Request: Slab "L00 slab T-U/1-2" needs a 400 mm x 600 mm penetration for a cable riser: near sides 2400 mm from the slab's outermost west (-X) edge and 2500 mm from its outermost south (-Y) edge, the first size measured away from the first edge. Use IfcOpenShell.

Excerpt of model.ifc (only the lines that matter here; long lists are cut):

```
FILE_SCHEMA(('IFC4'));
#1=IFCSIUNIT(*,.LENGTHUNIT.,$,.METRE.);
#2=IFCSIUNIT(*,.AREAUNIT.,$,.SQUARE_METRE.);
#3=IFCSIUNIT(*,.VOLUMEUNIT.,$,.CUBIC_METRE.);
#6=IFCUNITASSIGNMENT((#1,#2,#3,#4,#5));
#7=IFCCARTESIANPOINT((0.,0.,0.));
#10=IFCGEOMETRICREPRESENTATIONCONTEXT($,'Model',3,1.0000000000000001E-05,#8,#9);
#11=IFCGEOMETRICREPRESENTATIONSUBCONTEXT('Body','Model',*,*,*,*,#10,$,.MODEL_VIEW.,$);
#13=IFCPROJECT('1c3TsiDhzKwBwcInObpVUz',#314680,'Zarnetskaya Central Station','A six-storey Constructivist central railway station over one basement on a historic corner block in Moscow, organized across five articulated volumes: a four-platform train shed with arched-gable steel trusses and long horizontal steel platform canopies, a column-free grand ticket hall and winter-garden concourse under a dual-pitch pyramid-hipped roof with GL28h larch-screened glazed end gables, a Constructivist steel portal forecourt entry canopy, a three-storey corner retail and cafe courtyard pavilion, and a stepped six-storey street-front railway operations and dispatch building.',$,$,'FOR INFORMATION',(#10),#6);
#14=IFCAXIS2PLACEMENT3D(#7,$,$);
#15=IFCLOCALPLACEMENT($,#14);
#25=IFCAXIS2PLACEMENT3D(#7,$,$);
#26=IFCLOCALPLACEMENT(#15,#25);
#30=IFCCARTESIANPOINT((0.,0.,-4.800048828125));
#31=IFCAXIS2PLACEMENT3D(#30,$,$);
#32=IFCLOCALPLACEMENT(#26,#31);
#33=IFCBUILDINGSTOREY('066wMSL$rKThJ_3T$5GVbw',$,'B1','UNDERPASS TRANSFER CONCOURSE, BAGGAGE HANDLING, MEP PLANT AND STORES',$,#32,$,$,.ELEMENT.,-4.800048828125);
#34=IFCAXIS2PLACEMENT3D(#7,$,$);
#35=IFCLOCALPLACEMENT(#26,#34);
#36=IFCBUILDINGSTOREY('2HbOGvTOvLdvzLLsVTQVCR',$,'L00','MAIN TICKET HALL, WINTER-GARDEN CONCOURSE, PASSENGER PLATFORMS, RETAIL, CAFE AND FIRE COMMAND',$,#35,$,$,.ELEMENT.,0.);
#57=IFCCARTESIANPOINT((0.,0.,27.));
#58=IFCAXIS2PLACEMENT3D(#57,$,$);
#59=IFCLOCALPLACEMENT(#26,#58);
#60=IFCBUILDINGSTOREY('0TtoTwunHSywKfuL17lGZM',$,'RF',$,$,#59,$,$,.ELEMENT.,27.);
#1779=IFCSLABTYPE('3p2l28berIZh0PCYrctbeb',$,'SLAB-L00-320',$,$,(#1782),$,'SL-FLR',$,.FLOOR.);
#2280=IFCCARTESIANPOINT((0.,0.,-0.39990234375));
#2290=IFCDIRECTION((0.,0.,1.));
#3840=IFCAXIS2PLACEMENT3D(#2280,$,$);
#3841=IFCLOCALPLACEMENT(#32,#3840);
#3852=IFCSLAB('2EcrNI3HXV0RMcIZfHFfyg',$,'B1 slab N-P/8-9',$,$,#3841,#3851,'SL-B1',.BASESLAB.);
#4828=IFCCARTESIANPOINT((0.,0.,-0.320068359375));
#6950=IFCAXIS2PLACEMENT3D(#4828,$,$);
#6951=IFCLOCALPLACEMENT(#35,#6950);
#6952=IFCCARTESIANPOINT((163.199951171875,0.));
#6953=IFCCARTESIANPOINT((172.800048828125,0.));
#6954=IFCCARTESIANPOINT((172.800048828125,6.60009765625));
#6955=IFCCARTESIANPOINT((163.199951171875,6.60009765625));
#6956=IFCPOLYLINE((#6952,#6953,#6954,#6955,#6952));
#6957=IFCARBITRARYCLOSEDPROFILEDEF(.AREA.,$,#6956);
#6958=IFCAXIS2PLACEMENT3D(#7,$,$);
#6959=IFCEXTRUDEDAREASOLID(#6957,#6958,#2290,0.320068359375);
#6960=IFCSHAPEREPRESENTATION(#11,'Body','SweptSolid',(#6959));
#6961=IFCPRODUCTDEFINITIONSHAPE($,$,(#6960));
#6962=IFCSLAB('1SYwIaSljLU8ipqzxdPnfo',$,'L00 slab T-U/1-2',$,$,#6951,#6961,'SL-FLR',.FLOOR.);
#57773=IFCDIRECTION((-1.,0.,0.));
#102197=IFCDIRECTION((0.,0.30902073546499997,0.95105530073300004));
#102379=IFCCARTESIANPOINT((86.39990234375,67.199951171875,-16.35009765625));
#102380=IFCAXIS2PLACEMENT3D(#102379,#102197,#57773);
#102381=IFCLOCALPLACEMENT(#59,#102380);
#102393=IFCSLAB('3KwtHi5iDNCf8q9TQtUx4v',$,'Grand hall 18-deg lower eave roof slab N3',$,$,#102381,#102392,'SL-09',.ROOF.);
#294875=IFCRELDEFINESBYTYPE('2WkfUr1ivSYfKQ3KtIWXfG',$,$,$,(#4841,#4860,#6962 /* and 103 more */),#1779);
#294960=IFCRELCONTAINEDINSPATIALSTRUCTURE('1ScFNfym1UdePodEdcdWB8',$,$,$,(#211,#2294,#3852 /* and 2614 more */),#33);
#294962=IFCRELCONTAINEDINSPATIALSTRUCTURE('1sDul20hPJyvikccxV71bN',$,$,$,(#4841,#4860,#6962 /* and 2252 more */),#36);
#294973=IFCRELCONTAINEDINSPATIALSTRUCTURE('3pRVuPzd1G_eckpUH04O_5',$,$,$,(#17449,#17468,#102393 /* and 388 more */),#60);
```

```python
import numpy as np
import ifcopenshell
import ifcopenshell.api.feature
import ifcopenshell.api.geometry
import ifcopenshell.api.root
import ifcopenshell.geom
import ifcopenshell.util.placement
import ifcopenshell.util.representation
import ifcopenshell.util.shape
import ifcopenshell.util.unit

model = ifcopenshell.open("model.ifc")
unit_scale = ifcopenshell.util.unit.calculate_unit_scale(model)
settings = ifcopenshell.geom.settings()


def volume(element):
    """Net volume in cubic metres, openings subtracted."""
    shape = ifcopenshell.geom.create_shape(settings, element)
    return ifcopenshell.util.shape.get_volume(shape.geometry)


slab = model.by_guid("1SYwIaSljLU8ipqzxdPnfo")
before = volume(slab)

# Extent in the slab's own axes, in metres. The edges named are its -X and -Y sides.
slab_shape = ifcopenshell.geom.create_shape(settings, slab)
vertices = ifcopenshell.util.shape.get_vertices(slab_shape.geometry)
x_min, y_min, bottom = vertices.min(axis=0)
top = vertices[:, 2].max()

opening = ifcopenshell.api.root.create_entity(model, ifc_class="IfcOpeningElement", name="Cable riser opening", predefined_type="OPENING")
context = ifcopenshell.util.representation.get_context(model, "Model", "Body", "MODEL_VIEW")
width, depth = 0.4, 0.6
outline = [(0.0, 0.0), (width, 0.0), (width, depth), (0.0, depth), (0.0, 0.0)]
# Overshoot both faces by 50 mm so the cut is clean.
shape = ifcopenshell.api.geometry.add_slab_representation(
    model, context=context, depth=top - bottom + 0.1, polyline=outline
)
ifcopenshell.api.geometry.assign_representation(model, product=opening, representation=shape)

matrix = ifcopenshell.util.placement.get_local_placement(slab.ObjectPlacement)
matrix[:, 3] = matrix @ np.append(np.array([x_min + 2.4, y_min + 2.5, bottom - 0.05]) / unit_scale, 1.0)
ifcopenshell.api.geometry.edit_object_placement(model, product=opening, matrix=matrix, is_si=False)
ifcopenshell.api.feature.add_feature(model, feature=opening, element=slab)

after = volume(slab)

print(f"slab volume {before:.3f} -> {after:.3f} m3")

model.write("model_rev.ifc")
```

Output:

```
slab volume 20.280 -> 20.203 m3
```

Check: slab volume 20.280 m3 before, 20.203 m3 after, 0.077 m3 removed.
